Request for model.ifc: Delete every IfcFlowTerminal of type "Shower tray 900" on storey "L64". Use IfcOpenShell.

First a look at what the model holds.

```python
import ifcopenshell
import ifcopenshell.util.element

model = ifcopenshell.open("model.ifc")
print(model.schema)
storey = next(s for s in model.by_type("IfcBuildingStorey") if s.Name == "L64")
terminals = [e for e in ifcopenshell.util.element.get_decomposition(storey) if e.is_a("IfcFlowTerminal")]
seen = {}
for e in terminals:
    element_type = ifcopenshell.util.element.get_type(e)
    name = element_type.Name if element_type not in (None, e) else None
    seen[name] = seen.get(name, 0) + 1
for name, count in sorted(seen.items(), key=str):
    print(count, "x", name)
```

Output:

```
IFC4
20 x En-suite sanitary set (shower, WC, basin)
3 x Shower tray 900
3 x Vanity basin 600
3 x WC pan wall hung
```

```python
import ifcopenshell
import ifcopenshell.api.root
import ifcopenshell.util.element

model = ifcopenshell.open("model.ifc")

storey = next(s for s in model.by_type("IfcBuildingStorey") if s.Name == "L64")
terminals = [e for e in ifcopenshell.util.element.get_decomposition(storey) if e.is_a("IfcFlowTerminal")]
targets = [e for e in terminals if (t := ifcopenshell.util.element.get_type(e)) not in (None, e) and t.Name == "Shower tray 900"]

for e in targets:
    ifcopenshell.api.root.remove_product(model, product=e)
print(len(targets), "removed")

model.write("model_v2.ifc")
```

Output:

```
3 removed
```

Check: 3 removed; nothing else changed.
